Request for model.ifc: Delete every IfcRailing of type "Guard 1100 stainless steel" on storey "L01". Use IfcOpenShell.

First a look at what the model holds.

```python
import ifcopenshell
import ifcopenshell.util.element

model = ifcopenshell.open("model.ifc")
print(model.schema)
storey = next(s for s in model.by_type("IfcBuildingStorey") if s.Name == "L01")
railings = [e for e in ifcopenshell.util.element.get_decomposition(storey) if e.is_a("IfcRailing")]
seen = {}
for e in railings:
    element_type = ifcopenshell.util.element.get_type(e)
    name = element_type.Name if element_type not in (None, e) else None
    seen[name] = seen.get(name, 0) + 1
for name, count in sorted(seen.items(), key=str):
    print(count, "x", name)
```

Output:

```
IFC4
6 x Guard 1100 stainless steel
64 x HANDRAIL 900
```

```python
import ifcopenshell
import ifcopenshell.api.root
import ifcopenshell.util.element

model = ifcopenshell.open("model.ifc")

storey = next(s for s in model.by_type("IfcBuildingStorey") if s.Name == "L01")
railings = [e for e in ifcopenshell.util.element.get_decomposition(storey) if e.is_a("IfcRailing")]
targets = [e for e in railings if (t := ifcopenshell.util.element.get_type(e)) not in (None, e) and t.Name == "Guard 1100 stainless steel"]

for e in targets:
    ifcopenshell.api.root.remove_product(model, product=e)
print(len(targets), "removed")

model.write("model_edited.ifc")
```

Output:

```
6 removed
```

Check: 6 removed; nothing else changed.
